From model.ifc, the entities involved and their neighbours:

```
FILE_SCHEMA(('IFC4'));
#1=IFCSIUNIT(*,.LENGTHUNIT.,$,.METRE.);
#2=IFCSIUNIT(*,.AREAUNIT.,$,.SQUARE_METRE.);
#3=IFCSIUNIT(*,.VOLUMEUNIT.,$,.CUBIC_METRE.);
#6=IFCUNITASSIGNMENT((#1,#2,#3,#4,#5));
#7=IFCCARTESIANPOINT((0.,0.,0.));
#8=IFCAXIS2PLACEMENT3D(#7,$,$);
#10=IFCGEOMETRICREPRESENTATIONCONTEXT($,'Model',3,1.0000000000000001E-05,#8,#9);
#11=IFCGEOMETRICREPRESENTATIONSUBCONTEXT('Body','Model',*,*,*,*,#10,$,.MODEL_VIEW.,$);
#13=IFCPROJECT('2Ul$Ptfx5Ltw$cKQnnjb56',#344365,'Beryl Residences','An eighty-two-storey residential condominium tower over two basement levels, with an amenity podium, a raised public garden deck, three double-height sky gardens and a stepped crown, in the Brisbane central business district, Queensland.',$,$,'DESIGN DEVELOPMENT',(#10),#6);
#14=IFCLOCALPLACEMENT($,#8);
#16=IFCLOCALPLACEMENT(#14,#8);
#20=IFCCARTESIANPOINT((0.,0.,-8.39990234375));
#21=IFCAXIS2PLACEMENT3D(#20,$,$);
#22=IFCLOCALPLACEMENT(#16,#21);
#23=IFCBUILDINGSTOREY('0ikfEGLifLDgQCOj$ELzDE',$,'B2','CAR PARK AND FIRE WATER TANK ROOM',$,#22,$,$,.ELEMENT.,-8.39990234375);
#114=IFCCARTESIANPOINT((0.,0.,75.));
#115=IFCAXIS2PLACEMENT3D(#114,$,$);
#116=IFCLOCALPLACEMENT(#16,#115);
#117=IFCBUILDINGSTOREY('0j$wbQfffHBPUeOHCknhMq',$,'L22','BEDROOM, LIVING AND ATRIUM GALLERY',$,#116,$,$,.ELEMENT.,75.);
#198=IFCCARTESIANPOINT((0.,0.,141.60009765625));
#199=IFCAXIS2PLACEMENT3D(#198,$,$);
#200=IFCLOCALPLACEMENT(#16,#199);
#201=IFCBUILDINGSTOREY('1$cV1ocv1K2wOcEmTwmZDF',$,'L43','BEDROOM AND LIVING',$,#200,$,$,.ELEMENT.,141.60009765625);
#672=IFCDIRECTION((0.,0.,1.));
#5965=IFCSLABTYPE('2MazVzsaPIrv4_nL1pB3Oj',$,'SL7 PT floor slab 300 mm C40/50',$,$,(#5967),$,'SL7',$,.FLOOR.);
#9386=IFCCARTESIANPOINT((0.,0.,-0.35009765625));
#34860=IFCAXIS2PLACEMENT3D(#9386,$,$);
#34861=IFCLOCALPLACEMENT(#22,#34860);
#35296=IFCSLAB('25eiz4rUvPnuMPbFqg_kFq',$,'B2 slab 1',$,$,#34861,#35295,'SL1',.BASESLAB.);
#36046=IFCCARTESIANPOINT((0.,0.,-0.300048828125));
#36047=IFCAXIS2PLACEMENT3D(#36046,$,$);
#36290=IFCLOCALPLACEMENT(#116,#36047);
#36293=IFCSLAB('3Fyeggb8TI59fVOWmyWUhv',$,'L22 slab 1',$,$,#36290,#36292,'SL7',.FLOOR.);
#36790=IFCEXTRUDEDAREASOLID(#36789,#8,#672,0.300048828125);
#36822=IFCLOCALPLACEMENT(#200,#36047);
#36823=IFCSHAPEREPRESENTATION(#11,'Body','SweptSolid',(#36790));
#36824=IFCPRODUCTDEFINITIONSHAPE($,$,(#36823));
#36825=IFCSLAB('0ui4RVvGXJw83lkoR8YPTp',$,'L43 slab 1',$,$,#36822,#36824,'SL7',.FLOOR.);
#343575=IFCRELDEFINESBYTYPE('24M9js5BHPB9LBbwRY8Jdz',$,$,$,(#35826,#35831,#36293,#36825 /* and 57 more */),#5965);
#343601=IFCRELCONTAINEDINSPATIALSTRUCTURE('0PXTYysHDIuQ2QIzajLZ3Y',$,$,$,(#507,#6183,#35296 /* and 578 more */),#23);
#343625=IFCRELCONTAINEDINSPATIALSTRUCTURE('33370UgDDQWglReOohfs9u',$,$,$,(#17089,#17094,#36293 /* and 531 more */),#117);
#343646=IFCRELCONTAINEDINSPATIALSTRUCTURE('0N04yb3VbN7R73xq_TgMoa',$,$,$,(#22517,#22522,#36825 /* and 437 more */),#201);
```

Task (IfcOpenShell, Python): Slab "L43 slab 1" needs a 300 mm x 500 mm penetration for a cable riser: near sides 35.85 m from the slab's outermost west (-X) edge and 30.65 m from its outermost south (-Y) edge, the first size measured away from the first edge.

```python
import numpy as np
import ifcopenshell
import ifcopenshell.api.feature
import ifcopenshell.api.geometry
import ifcopenshell.api.root
import ifcopenshell.geom
import ifcopenshell.util.placement
import ifcopenshell.util.representation
import ifcopenshell.util.shape
import ifcopenshell.util.unit

model = ifcopenshell.open("model.ifc")
unit_scale = ifcopenshell.util.unit.calculate_unit_scale(model)
settings = ifcopenshell.geom.settings()


def volume(element):
    """Net volume in cubic metres, openings subtracted."""
    shape = ifcopenshell.geom.create_shape(settings, element)
    return ifcopenshell.util.shape.get_volume(shape.geometry)


slab = model.by_id(36825)
before = volume(slab)

# Extent in the slab's own axes, in metres. The edges named are its -X and -Y sides.
slab_shape = ifcopenshell.geom.create_shape(settings, slab)
vertices = ifcopenshell.util.shape.get_vertices(slab_shape.geometry)
x_min, y_min, bottom = vertices.min(axis=0)
top = vertices[:, 2].max()

opening = ifcopenshell.api.root.create_entity(model, ifc_class="IfcOpeningElement", name="Cable riser opening", predefined_type="OPENING")
context = ifcopenshell.util.representation.get_context(model, "Model", "Body", "MODEL_VIEW")
width, depth = 0.3, 0.5
outline = [(0.0, 0.0), (width, 0.0), (width, depth), (0.0, depth), (0.0, 0.0)]
# Overshoot both faces by 50 mm so the cut is clean.
shape = ifcopenshell.api.geometry.add_slab_representation(
    model, context=context, depth=top - bottom + 0.1, polyline=outline
)
ifcopenshell.api.geometry.assign_representation(model, product=opening, representation=shape)

matrix = ifcopenshell.util.placement.get_local_placement(slab.ObjectPlacement)
matrix[:, 3] = matrix @ np.append(np.array([x_min + 35.85, y_min + 30.65, bottom - 0.05]) / unit_scale, 1.0)
ifcopenshell.api.geometry.edit_object_placement(model, product=opening, matrix=matrix, is_si=False)
ifcopenshell.api.feature.add_feature(model, feature=opening, element=slab)

after = volume(slab)

print(f"slab volume {before:.3f} -> {after:.3f} m3")

model.write("model_edited.ifc")
```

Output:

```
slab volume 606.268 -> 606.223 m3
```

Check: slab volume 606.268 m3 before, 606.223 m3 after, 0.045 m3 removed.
